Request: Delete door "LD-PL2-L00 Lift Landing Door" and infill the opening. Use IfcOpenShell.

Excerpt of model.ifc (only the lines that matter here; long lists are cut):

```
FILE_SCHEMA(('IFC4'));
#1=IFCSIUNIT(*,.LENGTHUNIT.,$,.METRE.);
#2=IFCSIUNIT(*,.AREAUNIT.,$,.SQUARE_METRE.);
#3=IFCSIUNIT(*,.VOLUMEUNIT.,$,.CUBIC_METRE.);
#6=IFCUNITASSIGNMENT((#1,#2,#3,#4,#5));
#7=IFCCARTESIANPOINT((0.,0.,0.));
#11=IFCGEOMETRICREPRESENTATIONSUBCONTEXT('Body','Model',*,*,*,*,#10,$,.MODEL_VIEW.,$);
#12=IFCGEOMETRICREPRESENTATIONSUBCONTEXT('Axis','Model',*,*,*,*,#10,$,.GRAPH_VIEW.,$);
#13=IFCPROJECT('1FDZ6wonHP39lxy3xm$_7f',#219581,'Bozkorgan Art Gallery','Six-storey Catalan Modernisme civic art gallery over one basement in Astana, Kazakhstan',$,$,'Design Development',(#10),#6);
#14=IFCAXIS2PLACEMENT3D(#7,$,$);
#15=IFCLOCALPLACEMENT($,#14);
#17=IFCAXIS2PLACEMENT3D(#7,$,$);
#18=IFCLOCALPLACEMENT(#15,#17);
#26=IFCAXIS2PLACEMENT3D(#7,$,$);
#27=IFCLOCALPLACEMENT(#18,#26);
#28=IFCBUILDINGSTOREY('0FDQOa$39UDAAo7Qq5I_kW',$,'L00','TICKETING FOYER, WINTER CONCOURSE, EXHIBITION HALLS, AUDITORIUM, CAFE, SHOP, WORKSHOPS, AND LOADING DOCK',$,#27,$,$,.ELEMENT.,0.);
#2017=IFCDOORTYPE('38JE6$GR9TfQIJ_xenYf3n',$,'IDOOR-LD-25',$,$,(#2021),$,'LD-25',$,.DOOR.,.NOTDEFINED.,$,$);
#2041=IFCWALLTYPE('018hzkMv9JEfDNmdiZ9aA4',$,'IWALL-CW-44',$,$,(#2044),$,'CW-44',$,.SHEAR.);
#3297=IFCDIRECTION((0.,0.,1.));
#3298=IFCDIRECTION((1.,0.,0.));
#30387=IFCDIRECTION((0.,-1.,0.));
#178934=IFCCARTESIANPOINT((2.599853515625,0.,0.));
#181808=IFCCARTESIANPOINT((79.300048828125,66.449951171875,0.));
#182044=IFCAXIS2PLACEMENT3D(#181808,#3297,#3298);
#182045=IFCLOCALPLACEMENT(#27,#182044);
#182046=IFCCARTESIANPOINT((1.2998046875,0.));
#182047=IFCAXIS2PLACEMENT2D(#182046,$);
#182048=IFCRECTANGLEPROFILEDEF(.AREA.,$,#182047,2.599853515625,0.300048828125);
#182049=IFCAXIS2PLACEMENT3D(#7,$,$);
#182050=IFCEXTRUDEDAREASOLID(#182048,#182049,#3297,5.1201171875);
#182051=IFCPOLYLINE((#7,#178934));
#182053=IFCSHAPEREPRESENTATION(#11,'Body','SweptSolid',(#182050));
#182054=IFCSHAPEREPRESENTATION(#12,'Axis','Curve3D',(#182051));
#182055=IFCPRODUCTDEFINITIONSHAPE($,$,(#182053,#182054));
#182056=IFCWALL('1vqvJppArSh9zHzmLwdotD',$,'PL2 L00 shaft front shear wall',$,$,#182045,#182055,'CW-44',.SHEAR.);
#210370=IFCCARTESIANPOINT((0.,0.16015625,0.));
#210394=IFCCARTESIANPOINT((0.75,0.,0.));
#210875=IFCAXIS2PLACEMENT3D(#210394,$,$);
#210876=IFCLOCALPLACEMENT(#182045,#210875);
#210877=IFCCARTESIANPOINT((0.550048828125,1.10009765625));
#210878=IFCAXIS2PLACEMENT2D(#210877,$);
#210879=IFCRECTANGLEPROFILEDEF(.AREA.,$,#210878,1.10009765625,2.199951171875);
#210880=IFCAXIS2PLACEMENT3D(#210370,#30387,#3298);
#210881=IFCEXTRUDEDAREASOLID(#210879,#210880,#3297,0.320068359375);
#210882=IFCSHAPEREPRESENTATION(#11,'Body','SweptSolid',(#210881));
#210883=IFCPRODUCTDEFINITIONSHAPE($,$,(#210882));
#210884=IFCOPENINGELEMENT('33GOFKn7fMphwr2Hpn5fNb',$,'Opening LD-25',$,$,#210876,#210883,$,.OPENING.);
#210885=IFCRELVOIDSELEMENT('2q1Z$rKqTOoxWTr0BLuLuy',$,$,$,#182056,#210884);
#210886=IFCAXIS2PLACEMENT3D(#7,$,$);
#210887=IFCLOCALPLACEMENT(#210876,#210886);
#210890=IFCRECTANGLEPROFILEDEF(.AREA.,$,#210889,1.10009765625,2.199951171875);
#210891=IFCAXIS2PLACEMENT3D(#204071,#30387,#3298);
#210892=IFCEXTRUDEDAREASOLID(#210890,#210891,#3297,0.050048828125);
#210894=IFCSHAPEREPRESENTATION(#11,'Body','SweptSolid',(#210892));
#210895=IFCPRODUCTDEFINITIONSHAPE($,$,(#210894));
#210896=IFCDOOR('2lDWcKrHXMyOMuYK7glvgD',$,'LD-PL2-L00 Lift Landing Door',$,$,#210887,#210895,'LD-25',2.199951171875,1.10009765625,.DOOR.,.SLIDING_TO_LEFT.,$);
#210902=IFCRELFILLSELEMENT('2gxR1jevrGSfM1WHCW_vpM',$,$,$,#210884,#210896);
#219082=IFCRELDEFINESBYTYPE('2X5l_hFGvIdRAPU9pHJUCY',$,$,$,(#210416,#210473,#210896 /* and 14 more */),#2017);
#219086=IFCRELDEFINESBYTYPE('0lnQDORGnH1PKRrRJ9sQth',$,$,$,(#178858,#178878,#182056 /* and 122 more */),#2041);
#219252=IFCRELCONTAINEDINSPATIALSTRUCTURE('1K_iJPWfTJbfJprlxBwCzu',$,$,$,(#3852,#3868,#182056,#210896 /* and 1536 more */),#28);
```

```python
import ifcopenshell
import ifcopenshell.api.feature
import ifcopenshell.api.root
import ifcopenshell.geom
import ifcopenshell.util.shape

model = ifcopenshell.open("model.ifc")
settings = ifcopenshell.geom.settings()


def volume(element):
    """Net volume in cubic metres, openings subtracted."""
    shape = ifcopenshell.geom.create_shape(settings, element)
    return ifcopenshell.util.shape.get_volume(shape.geometry)


door = model.by_guid("2lDWcKrHXMyOMuYK7glvgD")
opening = door.FillsVoids[0].RelatingOpeningElement
wall = opening.VoidsElements[0].RelatingBuildingElement
before = volume(wall)

ifcopenshell.api.root.remove_product(model, product=door)
ifcopenshell.api.feature.remove_feature(model, feature=opening)

after = volume(wall)

print(f"wall volume {before:.3f} -> {after:.3f} m3")

model.write("model_v2.ifc")
```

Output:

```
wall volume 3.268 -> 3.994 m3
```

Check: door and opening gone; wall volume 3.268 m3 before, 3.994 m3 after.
